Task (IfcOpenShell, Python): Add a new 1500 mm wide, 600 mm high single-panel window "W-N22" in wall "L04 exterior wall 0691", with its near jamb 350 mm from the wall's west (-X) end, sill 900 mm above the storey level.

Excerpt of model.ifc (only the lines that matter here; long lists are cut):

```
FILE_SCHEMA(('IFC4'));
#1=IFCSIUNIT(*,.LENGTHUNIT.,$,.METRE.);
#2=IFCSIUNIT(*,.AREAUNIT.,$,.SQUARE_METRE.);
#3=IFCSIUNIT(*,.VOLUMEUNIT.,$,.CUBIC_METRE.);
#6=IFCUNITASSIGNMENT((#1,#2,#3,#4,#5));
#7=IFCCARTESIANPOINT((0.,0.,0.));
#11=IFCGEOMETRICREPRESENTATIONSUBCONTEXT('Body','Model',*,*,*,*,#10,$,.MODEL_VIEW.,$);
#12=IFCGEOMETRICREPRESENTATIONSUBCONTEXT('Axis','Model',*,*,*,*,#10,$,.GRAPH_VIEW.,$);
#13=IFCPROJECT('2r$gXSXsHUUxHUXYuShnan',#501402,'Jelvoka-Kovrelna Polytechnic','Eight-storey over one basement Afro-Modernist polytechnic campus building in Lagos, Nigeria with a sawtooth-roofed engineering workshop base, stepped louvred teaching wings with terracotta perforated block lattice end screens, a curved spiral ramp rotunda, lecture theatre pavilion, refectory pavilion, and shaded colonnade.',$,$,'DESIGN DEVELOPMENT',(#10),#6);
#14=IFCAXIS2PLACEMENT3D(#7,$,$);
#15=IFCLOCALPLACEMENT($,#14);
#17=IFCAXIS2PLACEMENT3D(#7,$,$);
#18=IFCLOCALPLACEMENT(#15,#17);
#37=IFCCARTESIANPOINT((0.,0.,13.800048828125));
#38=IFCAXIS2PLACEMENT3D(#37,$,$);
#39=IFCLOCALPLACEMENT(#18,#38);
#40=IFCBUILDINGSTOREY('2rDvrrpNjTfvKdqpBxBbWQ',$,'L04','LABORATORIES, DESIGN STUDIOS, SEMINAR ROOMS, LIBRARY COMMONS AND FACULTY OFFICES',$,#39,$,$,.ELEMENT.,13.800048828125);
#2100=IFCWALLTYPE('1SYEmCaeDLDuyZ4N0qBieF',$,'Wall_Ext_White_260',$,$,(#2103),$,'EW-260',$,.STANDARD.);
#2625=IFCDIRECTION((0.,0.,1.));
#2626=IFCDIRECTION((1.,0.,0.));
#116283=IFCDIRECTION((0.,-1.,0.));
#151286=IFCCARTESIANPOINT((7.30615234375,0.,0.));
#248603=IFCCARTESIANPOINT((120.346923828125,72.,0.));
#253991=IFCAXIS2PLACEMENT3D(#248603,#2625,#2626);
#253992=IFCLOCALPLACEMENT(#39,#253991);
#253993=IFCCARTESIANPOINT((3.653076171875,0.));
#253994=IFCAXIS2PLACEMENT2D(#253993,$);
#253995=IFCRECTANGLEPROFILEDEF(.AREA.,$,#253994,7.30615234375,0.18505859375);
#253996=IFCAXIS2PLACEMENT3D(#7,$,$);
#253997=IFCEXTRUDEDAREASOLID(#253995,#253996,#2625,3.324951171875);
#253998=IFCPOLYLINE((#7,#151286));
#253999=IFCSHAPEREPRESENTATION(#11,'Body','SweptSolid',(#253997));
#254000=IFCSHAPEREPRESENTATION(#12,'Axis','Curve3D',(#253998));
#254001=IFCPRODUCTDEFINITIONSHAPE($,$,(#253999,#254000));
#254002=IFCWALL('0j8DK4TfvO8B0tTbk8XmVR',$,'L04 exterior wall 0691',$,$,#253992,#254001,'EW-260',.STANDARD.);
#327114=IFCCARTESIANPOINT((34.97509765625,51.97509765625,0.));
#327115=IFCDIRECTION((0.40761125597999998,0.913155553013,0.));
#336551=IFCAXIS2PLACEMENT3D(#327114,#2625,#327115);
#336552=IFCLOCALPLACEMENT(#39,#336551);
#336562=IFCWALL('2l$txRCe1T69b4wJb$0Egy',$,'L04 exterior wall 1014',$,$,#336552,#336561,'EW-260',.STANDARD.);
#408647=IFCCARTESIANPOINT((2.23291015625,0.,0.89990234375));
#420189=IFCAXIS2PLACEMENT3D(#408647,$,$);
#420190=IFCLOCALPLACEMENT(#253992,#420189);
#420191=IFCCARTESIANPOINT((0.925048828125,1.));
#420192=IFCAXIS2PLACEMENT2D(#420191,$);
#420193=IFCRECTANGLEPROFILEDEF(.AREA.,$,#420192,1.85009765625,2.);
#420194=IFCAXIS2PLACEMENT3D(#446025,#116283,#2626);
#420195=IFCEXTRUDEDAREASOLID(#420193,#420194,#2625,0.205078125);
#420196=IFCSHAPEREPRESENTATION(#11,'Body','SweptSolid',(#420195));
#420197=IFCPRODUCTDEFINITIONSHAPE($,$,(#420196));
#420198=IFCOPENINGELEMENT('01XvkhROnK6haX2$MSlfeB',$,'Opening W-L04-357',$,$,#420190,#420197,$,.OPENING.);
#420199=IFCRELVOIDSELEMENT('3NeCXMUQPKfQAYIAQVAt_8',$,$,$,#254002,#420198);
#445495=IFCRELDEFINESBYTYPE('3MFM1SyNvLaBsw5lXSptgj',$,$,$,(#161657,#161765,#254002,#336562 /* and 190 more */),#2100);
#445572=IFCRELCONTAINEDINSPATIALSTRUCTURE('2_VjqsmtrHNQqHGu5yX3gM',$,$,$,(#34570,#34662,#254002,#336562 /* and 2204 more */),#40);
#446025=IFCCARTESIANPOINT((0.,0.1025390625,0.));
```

```python
import numpy as np
import ifcopenshell
import ifcopenshell.api.feature
import ifcopenshell.api.geometry
import ifcopenshell.api.root
import ifcopenshell.api.spatial
import ifcopenshell.geom
import ifcopenshell.util.element
import ifcopenshell.util.placement
import ifcopenshell.util.representation
import ifcopenshell.util.shape
import ifcopenshell.util.unit

model = ifcopenshell.open("model.ifc")
unit_scale = ifcopenshell.util.unit.calculate_unit_scale(model)
settings = ifcopenshell.geom.settings()


def volume(element):
    """Net volume in cubic metres, openings subtracted."""
    shape = ifcopenshell.geom.create_shape(settings, element)
    return ifcopenshell.util.shape.get_volume(shape.geometry)


wall = model.by_guid("0j8DK4TfvO8B0tTbk8XmVR")
storey = ifcopenshell.util.element.get_container(wall, ifc_class="IfcBuildingStorey")
context = ifcopenshell.util.representation.get_context(model, "Model", "Body", "MODEL_VIEW")
before = volume(wall)

width, height, from_end, sill = 1.5, 0.6, 0.35, 0.9  # metres

# The wall runs along its own X axis, and the end named is its -X end.
wall_shape = ifcopenshell.geom.create_shape(settings, wall)
x, y, z = ifcopenshell.util.shape.get_vertices(wall_shape.geometry).T
start = x.min() + from_end
face, thickness = float(y.min()), float(y.max() - y.min())
wall_matrix = ifcopenshell.util.placement.get_local_placement(wall.ObjectPlacement)
level = ifcopenshell.util.placement.get_local_placement(storey.ObjectPlacement)[2, 3]


def in_wall(x, y):
    """Placement at x, y metres in the wall's axes, at sill height."""
    matrix = wall_matrix.copy()
    matrix[:, 3] = wall_matrix @ np.array([x / unit_scale, y / unit_scale, 0.0, 1.0])
    matrix[2, 3] = level + sill / unit_scale
    return matrix


# Opening: a box that overshoots both wall faces by 50 mm.
opening = ifcopenshell.api.root.create_entity(model, ifc_class="IfcOpeningElement", predefined_type="OPENING")
box = ifcopenshell.api.geometry.add_wall_representation(
    model, context=context, length=width, height=height, thickness=thickness + 0.1
)
ifcopenshell.api.geometry.assign_representation(model, product=opening, representation=box)
ifcopenshell.api.geometry.edit_object_placement(model, product=opening, matrix=in_wall(start, face - 0.05), is_si=False)
ifcopenshell.api.feature.add_feature(model, feature=opening, element=wall)

window = ifcopenshell.api.root.create_entity(model, ifc_class="IfcWindow", name="W-N22", predefined_type="WINDOW")
window.OverallWidth, window.OverallHeight = width / unit_scale, height / unit_scale
window.PartitioningType = "SINGLE_PANEL"
body = ifcopenshell.api.geometry.add_window_representation(
    model,
    context=context,
    overall_width=window.OverallWidth,
    overall_height=window.OverallHeight,
    partition_type="SINGLE_PANEL",
)
ifcopenshell.api.geometry.assign_representation(model, product=window, representation=body)
ifcopenshell.api.spatial.assign_container(model, products=[window], relating_structure=storey)
ifcopenshell.api.feature.add_filling(model, opening=opening, element=window)

# Centre the window in the wall's thickness.
ifcopenshell.api.geometry.edit_object_placement(model, product=window, matrix=in_wall(start, face), is_si=False)
window_shape = ifcopenshell.geom.create_shape(settings, window)
depth = ifcopenshell.util.shape.get_vertices(window_shape.geometry)[:, 1]
offset = face + thickness / 2 - (depth.min() + depth.max()) / 2
ifcopenshell.api.geometry.edit_object_placement(model, product=window, matrix=in_wall(start, offset), is_si=False)

after = volume(wall)

print(f"wall volume {before:.3f} -> {after:.3f} m3")

model.write("model_edited.ifc")
```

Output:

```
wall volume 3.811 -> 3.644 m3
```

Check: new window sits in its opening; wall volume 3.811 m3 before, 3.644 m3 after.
